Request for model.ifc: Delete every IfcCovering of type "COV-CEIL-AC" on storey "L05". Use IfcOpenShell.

First a look at what the model holds.

```python
import ifcopenshell
import ifcopenshell.util.element

model = ifcopenshell.open("model.ifc")
print(model.schema)
storey = next(s for s in model.by_type("IfcBuildingStorey") if s.Name == "L05")
coverings = [e for e in ifcopenshell.util.element.get_decomposition(storey) if e.is_a("IfcCovering")]
seen = {}
for e in coverings:
    element_type = ifcopenshell.util.element.get_type(e)
    name = element_type.Name if element_type not in (None, e) else None
    seen[name] = seen.get(name, 0) + 1
for name, count in sorted(seen.items(), key=str):
    print(count, "x", name)
```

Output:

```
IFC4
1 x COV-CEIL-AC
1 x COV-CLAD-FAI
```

```python
import ifcopenshell
import ifcopenshell.api.root
import ifcopenshell.util.element

model = ifcopenshell.open("model.ifc")

storey = next(s for s in model.by_type("IfcBuildingStorey") if s.Name == "L05")
coverings = [e for e in ifcopenshell.util.element.get_decomposition(storey) if e.is_a("IfcCovering")]
targets = [e for e in coverings if (t := ifcopenshell.util.element.get_type(e)) not in (None, e) and t.Name == "COV-CEIL-AC"]

for e in targets:
    ifcopenshell.api.root.remove_product(model, product=e)
print(len(targets), "removed")

model.write("model_updated.ifc")
```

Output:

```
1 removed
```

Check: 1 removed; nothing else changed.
